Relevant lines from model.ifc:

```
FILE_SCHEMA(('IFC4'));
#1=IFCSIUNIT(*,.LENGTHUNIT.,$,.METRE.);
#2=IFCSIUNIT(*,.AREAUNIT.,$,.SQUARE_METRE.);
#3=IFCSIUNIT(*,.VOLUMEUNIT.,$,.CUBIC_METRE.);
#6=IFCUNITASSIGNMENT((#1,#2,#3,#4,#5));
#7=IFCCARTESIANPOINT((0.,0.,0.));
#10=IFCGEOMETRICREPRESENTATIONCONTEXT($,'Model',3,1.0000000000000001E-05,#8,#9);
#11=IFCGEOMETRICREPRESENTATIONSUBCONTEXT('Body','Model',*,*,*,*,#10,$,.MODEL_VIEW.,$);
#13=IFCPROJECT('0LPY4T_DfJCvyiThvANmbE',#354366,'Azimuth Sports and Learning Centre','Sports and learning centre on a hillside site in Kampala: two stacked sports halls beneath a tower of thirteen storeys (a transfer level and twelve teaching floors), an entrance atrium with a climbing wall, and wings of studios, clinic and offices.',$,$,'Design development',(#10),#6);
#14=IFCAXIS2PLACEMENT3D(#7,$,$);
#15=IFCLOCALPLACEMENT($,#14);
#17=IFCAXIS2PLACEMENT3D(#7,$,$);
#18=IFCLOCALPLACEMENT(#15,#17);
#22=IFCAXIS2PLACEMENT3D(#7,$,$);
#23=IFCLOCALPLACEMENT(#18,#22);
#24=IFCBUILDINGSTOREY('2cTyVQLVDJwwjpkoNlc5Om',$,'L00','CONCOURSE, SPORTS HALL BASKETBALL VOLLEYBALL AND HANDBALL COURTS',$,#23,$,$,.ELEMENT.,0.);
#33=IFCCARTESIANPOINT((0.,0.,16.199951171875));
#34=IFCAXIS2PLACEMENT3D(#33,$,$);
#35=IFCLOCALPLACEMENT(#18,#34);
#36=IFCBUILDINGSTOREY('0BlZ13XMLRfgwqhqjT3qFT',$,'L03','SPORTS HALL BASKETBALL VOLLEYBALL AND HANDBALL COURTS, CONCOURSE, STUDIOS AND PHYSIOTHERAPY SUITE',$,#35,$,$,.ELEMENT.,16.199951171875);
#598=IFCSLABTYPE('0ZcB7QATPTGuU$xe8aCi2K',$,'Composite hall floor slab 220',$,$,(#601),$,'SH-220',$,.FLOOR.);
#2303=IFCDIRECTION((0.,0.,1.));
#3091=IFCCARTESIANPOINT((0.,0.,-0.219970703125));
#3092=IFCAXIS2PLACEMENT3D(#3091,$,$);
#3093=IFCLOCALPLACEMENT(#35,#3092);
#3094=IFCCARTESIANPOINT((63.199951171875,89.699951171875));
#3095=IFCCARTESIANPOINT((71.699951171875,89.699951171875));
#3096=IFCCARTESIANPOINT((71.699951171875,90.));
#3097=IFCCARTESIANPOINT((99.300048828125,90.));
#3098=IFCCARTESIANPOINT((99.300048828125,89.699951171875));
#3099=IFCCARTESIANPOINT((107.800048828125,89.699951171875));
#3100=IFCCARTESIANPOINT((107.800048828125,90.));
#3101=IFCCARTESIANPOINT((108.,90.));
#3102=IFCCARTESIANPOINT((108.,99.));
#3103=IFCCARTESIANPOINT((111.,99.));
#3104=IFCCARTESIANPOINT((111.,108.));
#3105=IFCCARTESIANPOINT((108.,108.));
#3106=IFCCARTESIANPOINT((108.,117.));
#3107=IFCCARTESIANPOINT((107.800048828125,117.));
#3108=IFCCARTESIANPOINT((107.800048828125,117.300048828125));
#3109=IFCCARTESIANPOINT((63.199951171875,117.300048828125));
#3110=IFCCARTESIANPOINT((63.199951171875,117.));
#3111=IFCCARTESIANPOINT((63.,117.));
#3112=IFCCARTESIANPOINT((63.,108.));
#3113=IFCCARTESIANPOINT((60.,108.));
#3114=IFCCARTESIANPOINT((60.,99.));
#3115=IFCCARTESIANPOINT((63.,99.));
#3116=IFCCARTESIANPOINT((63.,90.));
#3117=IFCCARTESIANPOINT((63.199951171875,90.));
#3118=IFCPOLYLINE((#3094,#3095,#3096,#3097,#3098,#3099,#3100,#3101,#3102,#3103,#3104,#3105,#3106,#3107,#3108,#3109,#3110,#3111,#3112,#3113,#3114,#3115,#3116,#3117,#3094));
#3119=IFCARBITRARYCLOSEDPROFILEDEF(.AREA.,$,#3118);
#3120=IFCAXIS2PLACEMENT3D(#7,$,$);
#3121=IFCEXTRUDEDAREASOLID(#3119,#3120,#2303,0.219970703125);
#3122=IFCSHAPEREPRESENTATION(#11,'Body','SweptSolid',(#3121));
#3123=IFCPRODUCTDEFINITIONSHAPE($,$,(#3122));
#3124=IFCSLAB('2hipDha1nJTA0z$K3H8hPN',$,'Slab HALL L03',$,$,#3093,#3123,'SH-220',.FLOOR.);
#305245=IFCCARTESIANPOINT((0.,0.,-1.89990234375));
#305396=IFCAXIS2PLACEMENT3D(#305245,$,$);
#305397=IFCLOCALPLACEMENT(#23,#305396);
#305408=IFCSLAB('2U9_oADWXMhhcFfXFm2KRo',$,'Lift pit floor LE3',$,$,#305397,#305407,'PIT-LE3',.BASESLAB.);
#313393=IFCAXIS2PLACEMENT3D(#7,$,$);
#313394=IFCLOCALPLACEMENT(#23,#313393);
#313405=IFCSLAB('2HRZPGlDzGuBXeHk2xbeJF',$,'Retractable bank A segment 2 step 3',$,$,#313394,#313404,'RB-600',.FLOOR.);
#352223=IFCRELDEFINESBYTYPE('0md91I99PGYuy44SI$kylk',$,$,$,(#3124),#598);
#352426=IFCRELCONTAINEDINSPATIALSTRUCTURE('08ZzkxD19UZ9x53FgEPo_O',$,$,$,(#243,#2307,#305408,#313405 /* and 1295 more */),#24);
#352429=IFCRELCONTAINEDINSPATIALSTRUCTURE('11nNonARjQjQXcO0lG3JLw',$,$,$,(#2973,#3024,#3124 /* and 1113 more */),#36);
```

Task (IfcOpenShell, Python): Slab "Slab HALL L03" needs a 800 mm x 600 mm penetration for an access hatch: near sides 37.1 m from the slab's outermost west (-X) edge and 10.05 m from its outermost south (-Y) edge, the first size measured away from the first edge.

```python
import numpy as np
import ifcopenshell
import ifcopenshell.api.feature
import ifcopenshell.api.geometry
import ifcopenshell.api.root
import ifcopenshell.geom
import ifcopenshell.util.placement
import ifcopenshell.util.representation
import ifcopenshell.util.shape
import ifcopenshell.util.unit

model = ifcopenshell.open("model.ifc")
unit_scale = ifcopenshell.util.unit.calculate_unit_scale(model)
settings = ifcopenshell.geom.settings()


def volume(element):
    """Net volume in cubic metres, openings subtracted."""
    shape = ifcopenshell.geom.create_shape(settings, element)
    return ifcopenshell.util.shape.get_volume(shape.geometry)


slab = model.by_id(3124)
before = volume(slab)

# Extent in the slab's own axes, in metres. The edges named are its -X and -Y sides.
slab_shape = ifcopenshell.geom.create_shape(settings, slab)
vertices = ifcopenshell.util.shape.get_vertices(slab_shape.geometry)
x_min, y_min, bottom = vertices.min(axis=0)
top = vertices[:, 2].max()

opening = ifcopenshell.api.root.create_entity(model, ifc_class="IfcOpeningElement", name="Access hatch opening", predefined_type="OPENING")
context = ifcopenshell.util.representation.get_context(model, "Model", "Body", "MODEL_VIEW")
width, depth = 0.8, 0.6
outline = [(0.0, 0.0), (width, 0.0), (width, depth), (0.0, depth), (0.0, 0.0)]
# Overshoot both faces by 50 mm so the cut is clean.
shape = ifcopenshell.api.geometry.add_slab_representation(
    model, context=context, depth=top - bottom + 0.1, polyline=outline
)
ifcopenshell.api.geometry.assign_representation(model, product=opening, representation=shape)

matrix = ifcopenshell.util.placement.get_local_placement(slab.ObjectPlacement)
matrix[:, 3] = matrix @ np.append(np.array([x_min + 37.1, y_min + 10.05, bottom - 0.05]) / unit_scale, 1.0)
ifcopenshell.api.geometry.edit_object_placement(model, product=opening, matrix=matrix, is_si=False)
ifcopenshell.api.feature.add_feature(model, feature=opening, element=slab)

after = volume(slab)

print(f"slab volume {before:.3f} -> {after:.3f} m3")

model.write("model_v2.ifc")
```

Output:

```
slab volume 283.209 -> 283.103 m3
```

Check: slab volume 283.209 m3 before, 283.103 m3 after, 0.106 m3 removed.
